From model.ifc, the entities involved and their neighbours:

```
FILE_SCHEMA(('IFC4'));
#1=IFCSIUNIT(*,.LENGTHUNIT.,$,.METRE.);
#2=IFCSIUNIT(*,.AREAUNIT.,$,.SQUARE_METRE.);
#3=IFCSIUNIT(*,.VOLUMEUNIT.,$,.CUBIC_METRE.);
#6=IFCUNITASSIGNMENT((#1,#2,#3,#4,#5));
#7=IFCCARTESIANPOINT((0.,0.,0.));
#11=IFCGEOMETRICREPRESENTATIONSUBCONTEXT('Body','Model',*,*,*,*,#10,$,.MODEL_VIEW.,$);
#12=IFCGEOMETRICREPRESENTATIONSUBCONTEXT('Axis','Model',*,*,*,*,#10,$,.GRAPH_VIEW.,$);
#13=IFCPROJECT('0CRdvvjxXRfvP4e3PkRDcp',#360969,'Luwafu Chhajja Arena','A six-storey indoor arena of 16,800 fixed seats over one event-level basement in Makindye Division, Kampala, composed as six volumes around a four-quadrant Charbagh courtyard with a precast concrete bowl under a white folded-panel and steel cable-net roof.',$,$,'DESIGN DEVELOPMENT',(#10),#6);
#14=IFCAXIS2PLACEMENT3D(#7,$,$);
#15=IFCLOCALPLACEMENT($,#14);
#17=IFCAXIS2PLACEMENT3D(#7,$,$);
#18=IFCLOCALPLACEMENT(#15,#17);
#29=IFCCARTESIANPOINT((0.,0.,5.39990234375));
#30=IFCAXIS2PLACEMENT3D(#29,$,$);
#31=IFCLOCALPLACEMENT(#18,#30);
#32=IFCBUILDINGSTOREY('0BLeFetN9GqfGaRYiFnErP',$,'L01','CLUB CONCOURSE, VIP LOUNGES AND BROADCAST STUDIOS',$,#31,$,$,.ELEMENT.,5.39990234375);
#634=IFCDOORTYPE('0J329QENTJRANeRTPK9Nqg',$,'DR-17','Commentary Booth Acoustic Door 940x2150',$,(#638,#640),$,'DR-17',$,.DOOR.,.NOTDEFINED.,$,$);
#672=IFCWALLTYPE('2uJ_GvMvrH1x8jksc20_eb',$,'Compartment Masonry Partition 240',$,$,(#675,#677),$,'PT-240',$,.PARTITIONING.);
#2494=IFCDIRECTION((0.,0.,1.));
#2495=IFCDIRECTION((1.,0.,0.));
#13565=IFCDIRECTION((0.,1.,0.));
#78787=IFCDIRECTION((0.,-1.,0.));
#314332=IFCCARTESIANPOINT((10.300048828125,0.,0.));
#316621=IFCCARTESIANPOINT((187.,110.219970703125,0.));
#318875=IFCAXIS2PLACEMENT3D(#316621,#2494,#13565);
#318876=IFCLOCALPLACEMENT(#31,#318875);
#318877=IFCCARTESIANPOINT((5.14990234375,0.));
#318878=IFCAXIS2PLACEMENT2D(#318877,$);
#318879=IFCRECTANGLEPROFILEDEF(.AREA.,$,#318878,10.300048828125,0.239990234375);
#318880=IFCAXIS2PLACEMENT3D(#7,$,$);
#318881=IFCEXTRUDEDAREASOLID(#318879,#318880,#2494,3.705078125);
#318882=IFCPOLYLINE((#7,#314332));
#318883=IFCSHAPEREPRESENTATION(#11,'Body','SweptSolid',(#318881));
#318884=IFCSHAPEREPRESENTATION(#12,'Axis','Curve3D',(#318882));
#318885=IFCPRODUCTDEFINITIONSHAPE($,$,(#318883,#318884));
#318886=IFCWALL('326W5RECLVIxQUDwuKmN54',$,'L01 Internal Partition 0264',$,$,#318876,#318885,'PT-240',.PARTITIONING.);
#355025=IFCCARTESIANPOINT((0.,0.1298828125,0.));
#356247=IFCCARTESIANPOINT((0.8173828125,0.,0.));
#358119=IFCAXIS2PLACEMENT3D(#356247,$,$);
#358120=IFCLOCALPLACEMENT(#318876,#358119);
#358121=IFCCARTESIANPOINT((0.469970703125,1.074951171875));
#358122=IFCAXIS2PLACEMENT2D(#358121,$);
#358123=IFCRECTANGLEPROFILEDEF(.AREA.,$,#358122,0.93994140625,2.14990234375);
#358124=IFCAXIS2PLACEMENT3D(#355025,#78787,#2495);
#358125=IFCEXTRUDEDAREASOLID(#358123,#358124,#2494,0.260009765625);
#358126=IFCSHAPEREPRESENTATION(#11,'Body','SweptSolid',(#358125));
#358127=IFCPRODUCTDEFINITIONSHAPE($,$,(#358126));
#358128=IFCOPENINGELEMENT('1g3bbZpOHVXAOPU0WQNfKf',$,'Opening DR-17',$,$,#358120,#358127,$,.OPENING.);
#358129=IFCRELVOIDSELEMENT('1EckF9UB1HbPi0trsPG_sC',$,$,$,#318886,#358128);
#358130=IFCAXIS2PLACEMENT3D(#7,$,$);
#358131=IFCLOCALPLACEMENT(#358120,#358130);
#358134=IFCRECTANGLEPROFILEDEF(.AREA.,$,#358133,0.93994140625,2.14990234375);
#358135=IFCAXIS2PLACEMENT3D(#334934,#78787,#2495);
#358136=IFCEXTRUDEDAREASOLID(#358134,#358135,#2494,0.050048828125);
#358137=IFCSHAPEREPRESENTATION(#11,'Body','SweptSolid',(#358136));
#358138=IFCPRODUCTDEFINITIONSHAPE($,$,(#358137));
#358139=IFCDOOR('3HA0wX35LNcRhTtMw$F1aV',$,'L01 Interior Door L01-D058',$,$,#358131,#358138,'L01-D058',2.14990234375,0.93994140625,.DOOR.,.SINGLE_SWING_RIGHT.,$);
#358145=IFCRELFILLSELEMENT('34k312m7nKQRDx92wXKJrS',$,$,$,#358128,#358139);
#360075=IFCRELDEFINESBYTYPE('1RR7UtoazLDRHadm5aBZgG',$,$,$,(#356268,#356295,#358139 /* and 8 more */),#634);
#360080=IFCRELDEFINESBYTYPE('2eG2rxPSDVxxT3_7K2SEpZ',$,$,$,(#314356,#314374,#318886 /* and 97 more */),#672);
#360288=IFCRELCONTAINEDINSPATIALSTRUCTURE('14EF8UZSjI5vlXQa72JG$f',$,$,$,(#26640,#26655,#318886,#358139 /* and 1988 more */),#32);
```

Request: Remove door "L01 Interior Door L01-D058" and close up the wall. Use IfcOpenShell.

```python
import ifcopenshell
import ifcopenshell.api.feature
import ifcopenshell.api.root
import ifcopenshell.geom
import ifcopenshell.util.shape

model = ifcopenshell.open("model.ifc")
settings = ifcopenshell.geom.settings()


def volume(element):
    """Net volume in cubic metres, openings subtracted."""
    shape = ifcopenshell.geom.create_shape(settings, element)
    return ifcopenshell.util.shape.get_volume(shape.geometry)


door = model.by_id(358139)
opening = door.FillsVoids[0].RelatingOpeningElement
wall = opening.VoidsElements[0].RelatingBuildingElement
before = volume(wall)

ifcopenshell.api.root.remove_product(model, product=door)
ifcopenshell.api.feature.remove_feature(model, feature=opening)

after = volume(wall)

print(f"wall volume {before:.3f} -> {after:.3f} m3")

model.write("model_v2.ifc")
```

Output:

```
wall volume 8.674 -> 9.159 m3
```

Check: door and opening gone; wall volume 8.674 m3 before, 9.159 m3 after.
